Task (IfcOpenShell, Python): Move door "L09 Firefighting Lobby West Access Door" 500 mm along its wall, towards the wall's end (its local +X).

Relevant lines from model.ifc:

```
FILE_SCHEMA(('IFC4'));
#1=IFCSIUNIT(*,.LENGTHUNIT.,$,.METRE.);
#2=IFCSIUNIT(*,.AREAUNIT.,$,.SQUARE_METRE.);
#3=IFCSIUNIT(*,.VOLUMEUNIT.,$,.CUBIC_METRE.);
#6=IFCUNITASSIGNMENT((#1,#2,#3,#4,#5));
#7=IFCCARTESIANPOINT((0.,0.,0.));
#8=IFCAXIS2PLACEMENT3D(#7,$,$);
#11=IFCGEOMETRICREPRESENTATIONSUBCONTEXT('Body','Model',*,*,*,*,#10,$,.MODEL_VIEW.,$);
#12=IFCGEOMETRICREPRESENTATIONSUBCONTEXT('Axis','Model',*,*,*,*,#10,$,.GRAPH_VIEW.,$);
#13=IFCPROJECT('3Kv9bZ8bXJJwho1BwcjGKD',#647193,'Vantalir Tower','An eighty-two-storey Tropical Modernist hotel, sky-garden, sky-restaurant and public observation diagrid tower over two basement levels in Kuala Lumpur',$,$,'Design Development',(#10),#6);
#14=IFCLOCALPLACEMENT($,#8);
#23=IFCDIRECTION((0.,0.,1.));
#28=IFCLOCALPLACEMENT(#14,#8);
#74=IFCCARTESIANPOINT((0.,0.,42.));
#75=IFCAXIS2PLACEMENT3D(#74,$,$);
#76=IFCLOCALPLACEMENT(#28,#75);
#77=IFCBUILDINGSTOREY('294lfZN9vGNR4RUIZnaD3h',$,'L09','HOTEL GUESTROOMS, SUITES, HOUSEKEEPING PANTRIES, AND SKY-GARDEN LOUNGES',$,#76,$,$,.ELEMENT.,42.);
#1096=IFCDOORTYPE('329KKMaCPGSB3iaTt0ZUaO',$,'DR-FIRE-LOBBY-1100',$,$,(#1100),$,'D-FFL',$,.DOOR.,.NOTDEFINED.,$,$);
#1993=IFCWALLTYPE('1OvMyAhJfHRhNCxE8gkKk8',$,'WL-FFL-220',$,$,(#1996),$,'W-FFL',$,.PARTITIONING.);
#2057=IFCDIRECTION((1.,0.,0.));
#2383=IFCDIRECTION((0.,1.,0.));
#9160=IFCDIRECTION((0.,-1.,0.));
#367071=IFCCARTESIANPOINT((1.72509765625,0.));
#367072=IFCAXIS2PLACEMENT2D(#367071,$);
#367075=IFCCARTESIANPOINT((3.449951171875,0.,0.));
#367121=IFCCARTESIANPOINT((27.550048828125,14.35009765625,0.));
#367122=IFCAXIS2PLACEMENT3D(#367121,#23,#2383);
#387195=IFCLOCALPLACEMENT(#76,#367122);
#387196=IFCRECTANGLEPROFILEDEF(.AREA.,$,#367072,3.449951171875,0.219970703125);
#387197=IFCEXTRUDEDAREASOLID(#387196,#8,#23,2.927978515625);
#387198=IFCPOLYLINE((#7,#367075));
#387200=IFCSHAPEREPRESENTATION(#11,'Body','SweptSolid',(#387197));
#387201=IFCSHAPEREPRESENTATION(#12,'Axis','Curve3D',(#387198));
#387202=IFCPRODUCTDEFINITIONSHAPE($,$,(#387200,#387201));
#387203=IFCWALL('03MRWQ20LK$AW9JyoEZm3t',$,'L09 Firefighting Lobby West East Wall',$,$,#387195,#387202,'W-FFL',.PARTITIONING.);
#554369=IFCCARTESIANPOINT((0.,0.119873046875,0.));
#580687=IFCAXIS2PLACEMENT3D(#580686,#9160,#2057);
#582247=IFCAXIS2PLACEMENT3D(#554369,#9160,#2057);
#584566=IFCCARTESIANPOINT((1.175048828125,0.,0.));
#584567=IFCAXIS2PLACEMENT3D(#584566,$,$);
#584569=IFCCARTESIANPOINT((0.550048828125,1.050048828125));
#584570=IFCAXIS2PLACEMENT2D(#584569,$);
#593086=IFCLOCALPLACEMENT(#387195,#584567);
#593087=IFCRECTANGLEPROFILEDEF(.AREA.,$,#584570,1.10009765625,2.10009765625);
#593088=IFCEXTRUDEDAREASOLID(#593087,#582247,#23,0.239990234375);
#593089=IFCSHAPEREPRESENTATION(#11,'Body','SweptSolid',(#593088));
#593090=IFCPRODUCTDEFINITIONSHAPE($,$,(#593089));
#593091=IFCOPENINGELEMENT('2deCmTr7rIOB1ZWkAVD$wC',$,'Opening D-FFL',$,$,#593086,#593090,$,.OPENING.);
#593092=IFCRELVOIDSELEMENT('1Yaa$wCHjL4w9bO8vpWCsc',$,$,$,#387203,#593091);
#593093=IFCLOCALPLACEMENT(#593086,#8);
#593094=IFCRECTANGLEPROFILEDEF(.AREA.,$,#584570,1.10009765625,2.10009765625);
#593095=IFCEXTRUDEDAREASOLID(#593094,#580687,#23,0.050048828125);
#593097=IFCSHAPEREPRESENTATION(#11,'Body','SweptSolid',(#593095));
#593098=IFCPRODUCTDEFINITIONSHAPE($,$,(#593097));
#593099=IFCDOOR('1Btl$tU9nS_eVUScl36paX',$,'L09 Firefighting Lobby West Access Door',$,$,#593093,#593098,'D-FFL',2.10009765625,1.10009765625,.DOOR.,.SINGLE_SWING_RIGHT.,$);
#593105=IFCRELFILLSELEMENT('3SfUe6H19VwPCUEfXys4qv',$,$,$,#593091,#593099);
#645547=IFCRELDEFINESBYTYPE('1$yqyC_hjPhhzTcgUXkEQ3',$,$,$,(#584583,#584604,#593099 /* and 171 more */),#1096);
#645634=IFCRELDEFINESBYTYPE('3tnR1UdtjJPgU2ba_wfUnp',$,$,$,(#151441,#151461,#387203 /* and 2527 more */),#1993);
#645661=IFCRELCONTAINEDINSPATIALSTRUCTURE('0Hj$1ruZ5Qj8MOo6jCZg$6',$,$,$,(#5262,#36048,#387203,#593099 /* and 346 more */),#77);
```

```python
import ifcopenshell
import ifcopenshell.api.geometry
import ifcopenshell.util.placement
import ifcopenshell.util.unit

model = ifcopenshell.open("model.ifc")
unit_scale = ifcopenshell.util.unit.calculate_unit_scale(model)

door = model.by_id(593099)
opening = door.FillsVoids[0].RelatingOpeningElement
wall = opening.VoidsElements[0].RelatingBuildingElement

wall_matrix = ifcopenshell.util.placement.get_local_placement(wall.ObjectPlacement)
shift = wall_matrix[:3, 0] * 0.5 / unit_scale
before = ifcopenshell.util.placement.get_local_placement(door.ObjectPlacement)[:3, 3].copy()

# The door is placed relative to its opening, so it follows when the opening moves.
matrix = ifcopenshell.util.placement.get_local_placement(opening.ObjectPlacement)
matrix[:3, 3] += shift
ifcopenshell.api.geometry.edit_object_placement(
    model, product=opening, matrix=matrix, is_si=False, should_transform_children=True
)

after = ifcopenshell.util.placement.get_local_placement(door.ObjectPlacement)[:3, 3]
print("door moved by", (after - before).round(3) + 0.0)

model.write("model-out.ifc")
```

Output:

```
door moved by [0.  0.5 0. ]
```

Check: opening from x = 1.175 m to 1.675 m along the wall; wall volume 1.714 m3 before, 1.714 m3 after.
